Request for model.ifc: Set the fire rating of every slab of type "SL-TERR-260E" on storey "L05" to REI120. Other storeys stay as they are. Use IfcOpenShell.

First a look at what the model holds.

```python
import ifcopenshell
import ifcopenshell.util.element

model = ifcopenshell.open("model.ifc")
print(model.schema)
storey = next(s for s in model.by_type("IfcBuildingStorey") if s.Name == "L05")
slabs = [e for e in ifcopenshell.util.element.get_decomposition(storey) if e.is_a("IfcSlab")]
seen = {}
for e in slabs:
    element_type = ifcopenshell.util.element.get_type(e)
    key = (element_type.Name if element_type != e and element_type else None, ifcopenshell.util.element.get_pset(e, "Pset_SlabCommon", "FireRating"))
    seen[key] = seen.get(key, 0) + 1
for (name, value), count in sorted(seen.items(), key=str):
    print(count, "x", name, "|", value)
```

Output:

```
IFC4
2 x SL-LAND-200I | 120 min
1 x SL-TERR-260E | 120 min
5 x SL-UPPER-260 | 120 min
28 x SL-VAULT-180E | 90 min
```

```python
import ifcopenshell
import ifcopenshell.api.pset
import ifcopenshell.util.element

model = ifcopenshell.open("model.ifc")

storey = next(s for s in model.by_type("IfcBuildingStorey") if s.Name == "L05")
slabs = [e for e in ifcopenshell.util.element.get_decomposition(storey) if e.is_a("IfcSlab")]

count = 0
for e in slabs:
    element_type = ifcopenshell.util.element.get_type(e)
    if element_type in (None, e) or element_type.Name != "SL-TERR-260E":
        continue
    # add_pset returns the element's existing set when there is one.
    pset = ifcopenshell.api.pset.add_pset(model, product=e, name="Pset_SlabCommon")
    ifcopenshell.api.pset.edit_pset(model, pset=pset, properties={"FireRating": "REI120"})
    count += 1

print(count, "slabs updated")

model.write("model_updated.ifc")
```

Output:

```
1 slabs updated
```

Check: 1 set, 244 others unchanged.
